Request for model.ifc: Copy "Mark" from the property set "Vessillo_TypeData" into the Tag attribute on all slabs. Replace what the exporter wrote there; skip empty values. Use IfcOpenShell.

First a look at what the model holds.

```python
import ifcopenshell
import ifcopenshell.util.element

model = ifcopenshell.open("model.ifc")
print(model.schema)
slabs = model.by_type("IfcSlab")
print(len(slabs), "slabs")
for e in slabs[:8]:
    source = ifcopenshell.util.element.get_pset(e, "Vessillo_TypeData", "Mark")
    target = e.Tag
    print(e.id(), repr(source), repr(target), sep=" | ")
```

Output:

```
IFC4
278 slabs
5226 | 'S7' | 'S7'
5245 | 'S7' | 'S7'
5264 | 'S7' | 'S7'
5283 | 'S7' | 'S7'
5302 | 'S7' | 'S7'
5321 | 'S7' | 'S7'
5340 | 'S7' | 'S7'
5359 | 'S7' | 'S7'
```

```python
import ifcopenshell
import ifcopenshell.util.element

model = ifcopenshell.open("model.ifc")

count = 0
for e in model.by_type("IfcSlab"):
    value = ifcopenshell.util.element.get_pset(e, "Vessillo_TypeData", "Mark")
    current = e.Tag
    if not value or not value.strip() or current == value:
        continue
    e.Tag = value
    count += 1

print(count, "slabs updated")

model.write("model_v2.ifc")
```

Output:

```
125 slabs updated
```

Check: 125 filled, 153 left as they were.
